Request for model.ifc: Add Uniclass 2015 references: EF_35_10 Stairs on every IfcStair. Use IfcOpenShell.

First a look at what the model holds.

```python
import ifcopenshell

model = ifcopenshell.open("model.ifc")
print(model.schema)
print("classifications:", [c.Name for c in model.by_type("IfcClassification")])
for ifc_class in ("IfcDoor", "IfcRoof", "IfcStair", "IfcWall", "IfcWindow"):
    print(ifc_class, len(model.by_type(ifc_class)))
```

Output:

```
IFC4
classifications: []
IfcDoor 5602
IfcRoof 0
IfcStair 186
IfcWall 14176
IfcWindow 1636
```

```python
import ifcopenshell
import ifcopenshell.api.classification

model = ifcopenshell.open("model.ifc")

system = ifcopenshell.api.classification.add_classification(model, classification="Uniclass 2015")

codes = {
    "IfcStair": ("EF_35_10", "Stairs"),
}
for ifc_class, (code, name) in codes.items():
    products = model.by_type(ifc_class)
    ifcopenshell.api.classification.add_reference(
        model, products=products, classification=system, identification=code, name=name
    )
    print(code, len(products))

model.write("model_updated.ifc")
```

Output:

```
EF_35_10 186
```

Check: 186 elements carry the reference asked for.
